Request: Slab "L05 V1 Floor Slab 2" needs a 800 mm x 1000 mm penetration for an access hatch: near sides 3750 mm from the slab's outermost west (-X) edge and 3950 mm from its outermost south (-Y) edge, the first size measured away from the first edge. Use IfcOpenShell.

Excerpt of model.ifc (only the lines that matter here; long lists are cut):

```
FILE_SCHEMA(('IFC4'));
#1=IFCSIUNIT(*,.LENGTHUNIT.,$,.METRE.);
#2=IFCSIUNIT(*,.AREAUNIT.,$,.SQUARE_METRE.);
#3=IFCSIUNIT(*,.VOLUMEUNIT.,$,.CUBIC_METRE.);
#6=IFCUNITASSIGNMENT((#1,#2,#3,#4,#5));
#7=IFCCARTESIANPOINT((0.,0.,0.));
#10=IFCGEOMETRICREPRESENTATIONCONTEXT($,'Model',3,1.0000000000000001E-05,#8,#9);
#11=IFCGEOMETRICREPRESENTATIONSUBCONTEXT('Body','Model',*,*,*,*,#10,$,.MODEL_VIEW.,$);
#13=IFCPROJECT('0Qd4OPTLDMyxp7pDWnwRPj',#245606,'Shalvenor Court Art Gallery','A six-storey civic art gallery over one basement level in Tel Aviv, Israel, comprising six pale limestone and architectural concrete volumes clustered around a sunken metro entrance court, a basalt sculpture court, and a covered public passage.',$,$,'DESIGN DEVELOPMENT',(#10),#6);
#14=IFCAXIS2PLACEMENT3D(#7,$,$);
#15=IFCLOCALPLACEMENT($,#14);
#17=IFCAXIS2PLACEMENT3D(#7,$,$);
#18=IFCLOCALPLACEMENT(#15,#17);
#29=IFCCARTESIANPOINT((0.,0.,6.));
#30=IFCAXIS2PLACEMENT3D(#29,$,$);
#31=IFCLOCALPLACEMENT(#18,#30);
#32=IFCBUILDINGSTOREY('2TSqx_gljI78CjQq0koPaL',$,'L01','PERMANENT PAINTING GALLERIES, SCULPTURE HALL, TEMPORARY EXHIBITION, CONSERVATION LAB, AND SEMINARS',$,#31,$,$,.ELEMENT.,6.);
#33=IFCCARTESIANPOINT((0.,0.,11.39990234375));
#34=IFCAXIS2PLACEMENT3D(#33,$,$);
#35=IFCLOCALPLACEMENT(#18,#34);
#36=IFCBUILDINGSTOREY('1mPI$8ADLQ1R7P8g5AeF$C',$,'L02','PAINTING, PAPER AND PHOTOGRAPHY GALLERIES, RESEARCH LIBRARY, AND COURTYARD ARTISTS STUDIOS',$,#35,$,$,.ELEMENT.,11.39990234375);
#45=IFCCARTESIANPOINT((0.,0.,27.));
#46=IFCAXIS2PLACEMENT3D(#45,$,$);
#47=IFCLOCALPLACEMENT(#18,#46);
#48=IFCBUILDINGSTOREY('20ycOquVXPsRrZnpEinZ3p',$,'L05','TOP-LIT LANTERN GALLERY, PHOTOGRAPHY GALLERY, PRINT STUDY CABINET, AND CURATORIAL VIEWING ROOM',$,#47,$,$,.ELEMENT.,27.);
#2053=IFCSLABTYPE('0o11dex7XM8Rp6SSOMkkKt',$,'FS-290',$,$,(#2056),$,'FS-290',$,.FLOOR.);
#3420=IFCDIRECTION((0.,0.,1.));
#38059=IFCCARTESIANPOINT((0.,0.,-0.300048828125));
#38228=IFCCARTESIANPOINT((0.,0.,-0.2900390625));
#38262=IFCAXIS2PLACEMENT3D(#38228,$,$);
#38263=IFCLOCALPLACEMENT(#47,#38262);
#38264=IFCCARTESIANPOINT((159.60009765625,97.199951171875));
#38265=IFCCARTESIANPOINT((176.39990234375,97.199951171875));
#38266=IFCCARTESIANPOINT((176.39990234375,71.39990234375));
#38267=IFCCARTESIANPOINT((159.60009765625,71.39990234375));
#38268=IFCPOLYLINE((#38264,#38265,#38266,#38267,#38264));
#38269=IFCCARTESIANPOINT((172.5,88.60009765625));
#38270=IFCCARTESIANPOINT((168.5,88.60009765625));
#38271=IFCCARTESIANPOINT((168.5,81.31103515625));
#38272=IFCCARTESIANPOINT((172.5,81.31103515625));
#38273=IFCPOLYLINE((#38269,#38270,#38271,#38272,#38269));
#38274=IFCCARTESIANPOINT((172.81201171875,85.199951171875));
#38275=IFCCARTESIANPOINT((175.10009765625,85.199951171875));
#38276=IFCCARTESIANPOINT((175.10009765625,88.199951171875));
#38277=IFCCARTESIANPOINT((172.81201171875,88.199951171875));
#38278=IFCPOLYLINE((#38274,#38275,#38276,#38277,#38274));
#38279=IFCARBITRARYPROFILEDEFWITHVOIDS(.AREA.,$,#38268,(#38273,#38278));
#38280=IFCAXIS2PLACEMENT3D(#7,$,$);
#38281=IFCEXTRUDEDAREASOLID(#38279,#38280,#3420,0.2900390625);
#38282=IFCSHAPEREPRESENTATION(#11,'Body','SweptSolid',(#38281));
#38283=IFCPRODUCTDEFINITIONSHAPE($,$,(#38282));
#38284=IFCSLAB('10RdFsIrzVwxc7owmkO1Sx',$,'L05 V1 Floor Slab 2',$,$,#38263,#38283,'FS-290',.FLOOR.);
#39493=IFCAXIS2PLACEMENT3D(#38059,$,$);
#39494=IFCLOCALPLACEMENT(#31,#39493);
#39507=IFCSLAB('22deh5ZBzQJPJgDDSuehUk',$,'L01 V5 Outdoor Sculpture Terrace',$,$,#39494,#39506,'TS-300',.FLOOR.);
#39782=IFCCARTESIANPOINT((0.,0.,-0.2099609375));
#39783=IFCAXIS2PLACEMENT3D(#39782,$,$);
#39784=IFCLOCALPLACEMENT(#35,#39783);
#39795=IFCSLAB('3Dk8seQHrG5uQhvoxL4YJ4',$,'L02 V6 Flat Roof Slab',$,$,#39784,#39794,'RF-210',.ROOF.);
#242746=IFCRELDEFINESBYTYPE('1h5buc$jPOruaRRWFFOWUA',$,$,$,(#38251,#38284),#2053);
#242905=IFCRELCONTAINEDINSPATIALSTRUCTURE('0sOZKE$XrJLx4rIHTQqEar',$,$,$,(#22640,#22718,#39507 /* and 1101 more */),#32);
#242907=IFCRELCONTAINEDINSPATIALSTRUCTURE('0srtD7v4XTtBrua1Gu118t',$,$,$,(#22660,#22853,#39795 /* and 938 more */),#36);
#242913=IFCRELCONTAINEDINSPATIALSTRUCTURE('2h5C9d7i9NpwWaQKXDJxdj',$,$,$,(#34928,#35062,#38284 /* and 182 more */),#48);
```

```python
import numpy as np
import ifcopenshell
import ifcopenshell.api.feature
import ifcopenshell.api.geometry
import ifcopenshell.api.root
import ifcopenshell.geom
import ifcopenshell.util.placement
import ifcopenshell.util.representation
import ifcopenshell.util.shape
import ifcopenshell.util.unit

model = ifcopenshell.open("model.ifc")
unit_scale = ifcopenshell.util.unit.calculate_unit_scale(model)
settings = ifcopenshell.geom.settings()


def volume(element):
    """Net volume in cubic metres, openings subtracted."""
    shape = ifcopenshell.geom.create_shape(settings, element)
    return ifcopenshell.util.shape.get_volume(shape.geometry)


slab = model.by_guid("10RdFsIrzVwxc7owmkO1Sx")
before = volume(slab)

# Extent in the slab's own axes, in metres. The edges named are its -X and -Y sides.
slab_shape = ifcopenshell.geom.create_shape(settings, slab)
vertices = ifcopenshell.util.shape.get_vertices(slab_shape.geometry)
x_min, y_min, bottom = vertices.min(axis=0)
top = vertices[:, 2].max()

opening = ifcopenshell.api.root.create_entity(model, ifc_class="IfcOpeningElement", name="Access hatch opening", predefined_type="OPENING")
context = ifcopenshell.util.representation.get_context(model, "Model", "Body", "MODEL_VIEW")
width, depth = 0.8, 1
outline = [(0.0, 0.0), (width, 0.0), (width, depth), (0.0, depth), (0.0, 0.0)]
# Overshoot both faces by 50 mm so the cut is clean.
shape = ifcopenshell.api.geometry.add_slab_representation(
    model, context=context, depth=top - bottom + 0.1, polyline=outline
)
ifcopenshell.api.geometry.assign_representation(model, product=opening, representation=shape)

matrix = ifcopenshell.util.placement.get_local_placement(slab.ObjectPlacement)
matrix[:, 3] = matrix @ np.append(np.array([x_min + 3.75, y_min + 3.95, bottom - 0.05]) / unit_scale, 1.0)
ifcopenshell.api.geometry.edit_object_placement(model, product=opening, matrix=matrix, is_si=False)
ifcopenshell.api.feature.add_feature(model, feature=opening, element=slab)

after = volume(slab)

print(f"slab volume {before:.3f} -> {after:.3f} m3")

model.write("model_edited.ifc")
```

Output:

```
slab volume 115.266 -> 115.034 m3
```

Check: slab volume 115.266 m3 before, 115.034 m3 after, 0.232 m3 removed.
